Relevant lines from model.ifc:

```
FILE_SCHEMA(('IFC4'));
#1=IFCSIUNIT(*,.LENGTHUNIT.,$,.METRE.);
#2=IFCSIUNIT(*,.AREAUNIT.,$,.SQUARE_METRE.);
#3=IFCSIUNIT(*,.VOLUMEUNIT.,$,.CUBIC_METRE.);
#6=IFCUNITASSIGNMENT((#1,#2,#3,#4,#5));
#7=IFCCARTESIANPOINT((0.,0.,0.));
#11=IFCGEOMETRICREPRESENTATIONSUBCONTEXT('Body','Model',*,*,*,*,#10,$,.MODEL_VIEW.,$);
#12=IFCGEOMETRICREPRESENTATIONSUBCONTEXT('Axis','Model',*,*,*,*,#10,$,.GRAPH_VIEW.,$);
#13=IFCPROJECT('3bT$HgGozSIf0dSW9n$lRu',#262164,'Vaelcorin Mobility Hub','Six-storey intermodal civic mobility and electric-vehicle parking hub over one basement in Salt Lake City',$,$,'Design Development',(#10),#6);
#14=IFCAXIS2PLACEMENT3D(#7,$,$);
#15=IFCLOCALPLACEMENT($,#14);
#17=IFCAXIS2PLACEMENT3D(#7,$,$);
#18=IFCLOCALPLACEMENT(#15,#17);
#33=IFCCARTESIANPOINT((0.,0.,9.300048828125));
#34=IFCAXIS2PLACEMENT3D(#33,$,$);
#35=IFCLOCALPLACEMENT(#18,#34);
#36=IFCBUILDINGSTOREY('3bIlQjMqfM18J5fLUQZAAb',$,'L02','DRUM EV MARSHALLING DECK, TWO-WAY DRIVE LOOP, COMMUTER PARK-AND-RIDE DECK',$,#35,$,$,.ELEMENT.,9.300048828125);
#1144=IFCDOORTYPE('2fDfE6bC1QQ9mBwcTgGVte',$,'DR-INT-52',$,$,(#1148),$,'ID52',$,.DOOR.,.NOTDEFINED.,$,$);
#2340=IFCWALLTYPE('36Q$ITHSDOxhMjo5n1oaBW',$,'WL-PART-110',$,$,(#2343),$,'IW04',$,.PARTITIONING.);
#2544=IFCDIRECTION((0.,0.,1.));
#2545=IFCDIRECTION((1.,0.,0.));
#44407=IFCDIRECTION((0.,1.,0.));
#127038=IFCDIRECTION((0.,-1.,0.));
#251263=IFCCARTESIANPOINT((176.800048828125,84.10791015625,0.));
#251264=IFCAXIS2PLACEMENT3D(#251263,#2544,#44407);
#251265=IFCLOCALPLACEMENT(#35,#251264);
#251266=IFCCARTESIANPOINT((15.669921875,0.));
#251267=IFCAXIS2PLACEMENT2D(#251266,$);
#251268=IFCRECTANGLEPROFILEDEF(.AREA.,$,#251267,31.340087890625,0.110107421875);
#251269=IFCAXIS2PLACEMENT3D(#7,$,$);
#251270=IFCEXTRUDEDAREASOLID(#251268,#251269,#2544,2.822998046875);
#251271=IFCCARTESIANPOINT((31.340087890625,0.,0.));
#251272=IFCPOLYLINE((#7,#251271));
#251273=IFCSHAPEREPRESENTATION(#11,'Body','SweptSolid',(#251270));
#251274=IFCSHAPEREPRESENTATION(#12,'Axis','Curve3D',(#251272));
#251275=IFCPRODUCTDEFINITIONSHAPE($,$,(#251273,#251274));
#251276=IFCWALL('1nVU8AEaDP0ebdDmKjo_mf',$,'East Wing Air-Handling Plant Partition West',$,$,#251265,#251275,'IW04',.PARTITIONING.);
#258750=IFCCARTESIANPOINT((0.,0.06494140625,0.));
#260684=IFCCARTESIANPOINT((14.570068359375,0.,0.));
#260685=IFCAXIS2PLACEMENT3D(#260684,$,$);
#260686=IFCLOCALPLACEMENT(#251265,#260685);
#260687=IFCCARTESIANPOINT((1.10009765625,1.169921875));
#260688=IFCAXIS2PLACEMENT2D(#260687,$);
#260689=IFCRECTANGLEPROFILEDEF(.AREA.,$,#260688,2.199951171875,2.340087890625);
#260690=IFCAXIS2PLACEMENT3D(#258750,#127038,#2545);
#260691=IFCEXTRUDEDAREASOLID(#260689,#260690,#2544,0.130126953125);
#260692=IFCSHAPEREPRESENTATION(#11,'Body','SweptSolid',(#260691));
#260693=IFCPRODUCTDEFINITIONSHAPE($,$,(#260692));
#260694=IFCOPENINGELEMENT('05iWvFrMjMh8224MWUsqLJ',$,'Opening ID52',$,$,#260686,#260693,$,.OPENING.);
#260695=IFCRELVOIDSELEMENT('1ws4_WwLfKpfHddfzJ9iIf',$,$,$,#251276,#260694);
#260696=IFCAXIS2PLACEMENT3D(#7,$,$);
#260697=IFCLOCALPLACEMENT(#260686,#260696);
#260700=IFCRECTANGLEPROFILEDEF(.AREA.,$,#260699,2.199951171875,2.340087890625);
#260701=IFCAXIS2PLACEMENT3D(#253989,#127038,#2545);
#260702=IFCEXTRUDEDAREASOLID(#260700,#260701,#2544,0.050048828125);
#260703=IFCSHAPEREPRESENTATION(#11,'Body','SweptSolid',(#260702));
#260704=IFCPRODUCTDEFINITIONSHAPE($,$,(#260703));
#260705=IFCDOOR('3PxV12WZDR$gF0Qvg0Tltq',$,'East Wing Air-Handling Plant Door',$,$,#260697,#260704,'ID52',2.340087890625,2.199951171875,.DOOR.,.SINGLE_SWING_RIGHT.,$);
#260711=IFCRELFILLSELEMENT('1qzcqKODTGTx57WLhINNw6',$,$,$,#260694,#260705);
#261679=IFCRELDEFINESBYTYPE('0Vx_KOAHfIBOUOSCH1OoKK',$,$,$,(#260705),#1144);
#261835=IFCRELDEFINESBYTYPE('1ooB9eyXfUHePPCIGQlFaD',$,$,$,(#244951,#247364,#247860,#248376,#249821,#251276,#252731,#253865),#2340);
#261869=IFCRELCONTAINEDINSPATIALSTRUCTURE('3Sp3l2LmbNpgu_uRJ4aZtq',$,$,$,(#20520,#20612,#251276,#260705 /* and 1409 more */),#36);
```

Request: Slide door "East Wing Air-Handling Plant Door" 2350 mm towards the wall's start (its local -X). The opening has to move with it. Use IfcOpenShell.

```python
import ifcopenshell
import ifcopenshell.api.geometry
import ifcopenshell.util.placement

model = ifcopenshell.open("model.ifc")

door = model.by_guid("3PxV12WZDR$gF0Qvg0Tltq")
opening = door.FillsVoids[0].RelatingOpeningElement
wall = opening.VoidsElements[0].RelatingBuildingElement

wall_matrix = ifcopenshell.util.placement.get_local_placement(wall.ObjectPlacement)
shift = wall_matrix[:3, 0] * -2.35
before = ifcopenshell.util.placement.get_local_placement(door.ObjectPlacement)[:3, 3].copy()

# The door is placed relative to its opening, so it follows when the opening moves.
matrix = ifcopenshell.util.placement.get_local_placement(opening.ObjectPlacement)
matrix[:3, 3] += shift
ifcopenshell.api.geometry.edit_object_placement(
    model, product=opening, matrix=matrix, is_si=False, should_transform_children=True
)

after = ifcopenshell.util.placement.get_local_placement(door.ObjectPlacement)[:3, 3]
print("door moved by", (after - before).round(3) + 0.0)

model.write("model_v2.ifc")
```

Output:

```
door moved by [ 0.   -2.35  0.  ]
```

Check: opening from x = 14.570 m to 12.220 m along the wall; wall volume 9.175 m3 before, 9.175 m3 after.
